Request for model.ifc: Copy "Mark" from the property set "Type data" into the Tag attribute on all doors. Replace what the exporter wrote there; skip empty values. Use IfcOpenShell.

First a look at what the model holds.

```python
import ifcopenshell
import ifcopenshell.util.element

model = ifcopenshell.open("model.ifc")
print(model.schema)
doors = model.by_type("IfcDoor")
print(len(doors), "doors")
for e in doors[:8]:
    source = ifcopenshell.util.element.get_pset(e, "Type data", "Mark")
    target = e.Tag
    print(e.id(), repr(source), repr(target), sep=" | ")
```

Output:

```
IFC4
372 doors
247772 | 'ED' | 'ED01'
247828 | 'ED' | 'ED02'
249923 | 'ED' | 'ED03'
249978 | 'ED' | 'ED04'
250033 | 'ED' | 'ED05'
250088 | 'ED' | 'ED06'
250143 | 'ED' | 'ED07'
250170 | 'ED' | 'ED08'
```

```python
import ifcopenshell
import ifcopenshell.util.element

model = ifcopenshell.open("model.ifc")

count = 0
for e in model.by_type("IfcDoor"):
    value = ifcopenshell.util.element.get_pset(e, "Type data", "Mark")
    current = e.Tag
    if not value or not value.strip() or current == value:
        continue
    e.Tag = value
    count += 1

print(count, "doors updated")

model.write("model_edited.ifc")
```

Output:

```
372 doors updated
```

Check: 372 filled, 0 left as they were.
